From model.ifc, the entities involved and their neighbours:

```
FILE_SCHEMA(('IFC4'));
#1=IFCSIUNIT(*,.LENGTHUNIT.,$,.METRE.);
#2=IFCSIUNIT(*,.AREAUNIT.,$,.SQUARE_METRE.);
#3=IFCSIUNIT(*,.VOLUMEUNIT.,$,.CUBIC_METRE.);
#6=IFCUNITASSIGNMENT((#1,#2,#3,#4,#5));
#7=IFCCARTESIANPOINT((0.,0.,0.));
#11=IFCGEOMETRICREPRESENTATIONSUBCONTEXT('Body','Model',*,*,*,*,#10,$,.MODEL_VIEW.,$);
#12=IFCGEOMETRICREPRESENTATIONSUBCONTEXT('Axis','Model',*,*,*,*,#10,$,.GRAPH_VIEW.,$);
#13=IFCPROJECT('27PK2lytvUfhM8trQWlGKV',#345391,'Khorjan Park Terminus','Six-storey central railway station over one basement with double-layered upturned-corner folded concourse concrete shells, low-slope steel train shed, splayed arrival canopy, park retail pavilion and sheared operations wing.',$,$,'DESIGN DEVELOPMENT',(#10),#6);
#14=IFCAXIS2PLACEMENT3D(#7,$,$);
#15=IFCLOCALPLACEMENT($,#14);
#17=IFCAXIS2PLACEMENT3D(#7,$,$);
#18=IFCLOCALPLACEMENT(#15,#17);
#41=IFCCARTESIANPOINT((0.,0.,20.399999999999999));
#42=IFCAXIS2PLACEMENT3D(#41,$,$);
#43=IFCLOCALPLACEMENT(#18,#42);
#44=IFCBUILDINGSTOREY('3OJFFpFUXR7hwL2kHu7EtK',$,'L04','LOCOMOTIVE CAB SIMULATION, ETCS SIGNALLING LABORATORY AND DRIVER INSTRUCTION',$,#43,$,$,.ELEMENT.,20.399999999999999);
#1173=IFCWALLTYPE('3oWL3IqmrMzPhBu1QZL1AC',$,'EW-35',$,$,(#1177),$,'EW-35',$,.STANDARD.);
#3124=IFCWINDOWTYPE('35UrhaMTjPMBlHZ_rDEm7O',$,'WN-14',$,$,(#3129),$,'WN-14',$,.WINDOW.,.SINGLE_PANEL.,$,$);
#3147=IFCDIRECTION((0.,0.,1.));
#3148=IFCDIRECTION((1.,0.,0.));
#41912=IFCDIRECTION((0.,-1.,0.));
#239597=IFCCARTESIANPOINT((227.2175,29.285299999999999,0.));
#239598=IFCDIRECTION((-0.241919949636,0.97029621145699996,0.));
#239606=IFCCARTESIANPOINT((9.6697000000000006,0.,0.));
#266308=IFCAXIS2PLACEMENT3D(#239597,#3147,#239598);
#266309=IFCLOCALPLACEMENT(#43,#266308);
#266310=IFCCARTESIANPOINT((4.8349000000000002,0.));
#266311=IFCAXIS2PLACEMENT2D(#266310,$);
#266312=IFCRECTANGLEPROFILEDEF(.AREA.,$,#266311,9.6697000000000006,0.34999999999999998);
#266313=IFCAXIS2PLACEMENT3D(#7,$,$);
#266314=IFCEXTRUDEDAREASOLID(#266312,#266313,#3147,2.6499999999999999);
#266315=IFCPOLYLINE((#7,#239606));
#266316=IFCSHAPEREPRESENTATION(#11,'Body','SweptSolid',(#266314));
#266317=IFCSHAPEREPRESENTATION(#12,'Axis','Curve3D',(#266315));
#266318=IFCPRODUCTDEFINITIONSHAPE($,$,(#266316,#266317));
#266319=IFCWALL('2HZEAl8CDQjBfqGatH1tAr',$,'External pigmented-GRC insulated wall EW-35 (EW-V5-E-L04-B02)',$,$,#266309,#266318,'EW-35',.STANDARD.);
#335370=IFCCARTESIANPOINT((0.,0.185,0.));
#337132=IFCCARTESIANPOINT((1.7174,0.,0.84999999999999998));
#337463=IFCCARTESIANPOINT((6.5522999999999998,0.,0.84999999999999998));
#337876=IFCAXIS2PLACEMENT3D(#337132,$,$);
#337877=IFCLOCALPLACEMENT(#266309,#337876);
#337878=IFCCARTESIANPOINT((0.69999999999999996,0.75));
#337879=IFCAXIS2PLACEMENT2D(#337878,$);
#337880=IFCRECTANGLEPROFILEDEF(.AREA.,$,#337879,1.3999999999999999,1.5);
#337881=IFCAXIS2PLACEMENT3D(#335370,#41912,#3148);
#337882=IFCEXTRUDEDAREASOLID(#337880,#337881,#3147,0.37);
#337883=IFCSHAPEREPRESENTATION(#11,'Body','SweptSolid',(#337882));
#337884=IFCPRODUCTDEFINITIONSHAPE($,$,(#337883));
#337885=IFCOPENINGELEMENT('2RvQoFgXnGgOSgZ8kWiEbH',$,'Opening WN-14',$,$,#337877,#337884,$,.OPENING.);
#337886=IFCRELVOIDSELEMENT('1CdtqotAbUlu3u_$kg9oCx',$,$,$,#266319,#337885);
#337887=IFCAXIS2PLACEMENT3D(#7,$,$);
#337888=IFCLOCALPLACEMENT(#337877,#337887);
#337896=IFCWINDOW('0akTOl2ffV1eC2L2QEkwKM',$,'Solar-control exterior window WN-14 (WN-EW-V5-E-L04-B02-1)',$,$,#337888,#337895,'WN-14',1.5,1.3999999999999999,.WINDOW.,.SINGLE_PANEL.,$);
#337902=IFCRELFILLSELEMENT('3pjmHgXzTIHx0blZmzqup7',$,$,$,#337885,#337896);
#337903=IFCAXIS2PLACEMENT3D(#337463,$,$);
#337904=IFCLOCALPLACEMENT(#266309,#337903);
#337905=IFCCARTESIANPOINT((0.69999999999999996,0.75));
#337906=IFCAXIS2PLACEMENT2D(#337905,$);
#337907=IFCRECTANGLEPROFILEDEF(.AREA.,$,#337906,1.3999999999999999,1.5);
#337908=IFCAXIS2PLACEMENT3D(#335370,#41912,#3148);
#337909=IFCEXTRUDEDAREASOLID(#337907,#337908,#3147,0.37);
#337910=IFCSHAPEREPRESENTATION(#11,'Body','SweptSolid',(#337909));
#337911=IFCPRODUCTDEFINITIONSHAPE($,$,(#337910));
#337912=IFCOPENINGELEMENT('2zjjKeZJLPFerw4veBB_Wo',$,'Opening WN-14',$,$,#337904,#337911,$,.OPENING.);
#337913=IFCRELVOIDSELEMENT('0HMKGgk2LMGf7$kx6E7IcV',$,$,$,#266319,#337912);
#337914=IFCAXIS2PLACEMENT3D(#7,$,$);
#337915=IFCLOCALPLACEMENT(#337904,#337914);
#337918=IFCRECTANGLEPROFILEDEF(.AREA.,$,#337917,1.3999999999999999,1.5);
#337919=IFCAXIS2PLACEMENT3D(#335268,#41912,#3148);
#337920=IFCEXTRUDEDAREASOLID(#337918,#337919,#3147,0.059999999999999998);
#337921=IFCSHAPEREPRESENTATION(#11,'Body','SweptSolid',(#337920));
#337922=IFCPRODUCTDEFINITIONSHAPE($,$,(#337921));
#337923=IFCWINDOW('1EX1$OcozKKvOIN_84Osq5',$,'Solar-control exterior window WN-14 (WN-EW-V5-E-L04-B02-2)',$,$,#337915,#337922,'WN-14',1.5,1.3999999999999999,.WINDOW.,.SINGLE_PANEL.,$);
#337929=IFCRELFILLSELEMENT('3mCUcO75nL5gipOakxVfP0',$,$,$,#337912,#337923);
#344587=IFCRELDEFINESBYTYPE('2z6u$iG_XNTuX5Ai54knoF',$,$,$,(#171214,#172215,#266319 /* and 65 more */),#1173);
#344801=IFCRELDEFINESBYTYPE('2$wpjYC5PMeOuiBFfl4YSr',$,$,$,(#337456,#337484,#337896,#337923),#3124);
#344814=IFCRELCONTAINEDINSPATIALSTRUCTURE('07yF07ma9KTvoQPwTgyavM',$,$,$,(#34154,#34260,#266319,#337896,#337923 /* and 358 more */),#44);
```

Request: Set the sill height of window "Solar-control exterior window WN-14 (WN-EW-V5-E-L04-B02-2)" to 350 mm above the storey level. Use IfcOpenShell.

```python
import numpy as np
import ifcopenshell
import ifcopenshell.api.geometry
import ifcopenshell.geom
import ifcopenshell.util.element
import ifcopenshell.util.placement
import ifcopenshell.util.shape
import ifcopenshell.util.unit

model = ifcopenshell.open("model.ifc")
unit_scale = ifcopenshell.util.unit.calculate_unit_scale(model)

window = model.by_guid("1EX1$OcozKKvOIN_84Osq5")
opening = window.FillsVoids[0].RelatingOpeningElement
storey = ifcopenshell.util.element.get_container(window, ifc_class="IfcBuildingStorey")
level = ifcopenshell.util.placement.get_local_placement(storey.ObjectPlacement)[2, 3]

# The opening's origin need not be at the sill, so measure its lowest point.
shape = ifcopenshell.geom.create_shape(ifcopenshell.geom.settings(), opening)
bottom = ifcopenshell.util.shape.get_shape_bottom_elevation(shape, shape.geometry) / unit_scale
dz = level + 0.35 / unit_scale - bottom

shift = np.array([0.0, 0.0, dz])
# The window is placed relative to its opening, so it follows when the opening moves.
matrix = ifcopenshell.util.placement.get_local_placement(opening.ObjectPlacement)
matrix[:3, 3] += shift
ifcopenshell.api.geometry.edit_object_placement(
    model, product=opening, matrix=matrix, is_si=False, should_transform_children=True
)

print(f"moved by {dz * unit_scale:+.3f} m")

model.write("model_rev.ifc")
```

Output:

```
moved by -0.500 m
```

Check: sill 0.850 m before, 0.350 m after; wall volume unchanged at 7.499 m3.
